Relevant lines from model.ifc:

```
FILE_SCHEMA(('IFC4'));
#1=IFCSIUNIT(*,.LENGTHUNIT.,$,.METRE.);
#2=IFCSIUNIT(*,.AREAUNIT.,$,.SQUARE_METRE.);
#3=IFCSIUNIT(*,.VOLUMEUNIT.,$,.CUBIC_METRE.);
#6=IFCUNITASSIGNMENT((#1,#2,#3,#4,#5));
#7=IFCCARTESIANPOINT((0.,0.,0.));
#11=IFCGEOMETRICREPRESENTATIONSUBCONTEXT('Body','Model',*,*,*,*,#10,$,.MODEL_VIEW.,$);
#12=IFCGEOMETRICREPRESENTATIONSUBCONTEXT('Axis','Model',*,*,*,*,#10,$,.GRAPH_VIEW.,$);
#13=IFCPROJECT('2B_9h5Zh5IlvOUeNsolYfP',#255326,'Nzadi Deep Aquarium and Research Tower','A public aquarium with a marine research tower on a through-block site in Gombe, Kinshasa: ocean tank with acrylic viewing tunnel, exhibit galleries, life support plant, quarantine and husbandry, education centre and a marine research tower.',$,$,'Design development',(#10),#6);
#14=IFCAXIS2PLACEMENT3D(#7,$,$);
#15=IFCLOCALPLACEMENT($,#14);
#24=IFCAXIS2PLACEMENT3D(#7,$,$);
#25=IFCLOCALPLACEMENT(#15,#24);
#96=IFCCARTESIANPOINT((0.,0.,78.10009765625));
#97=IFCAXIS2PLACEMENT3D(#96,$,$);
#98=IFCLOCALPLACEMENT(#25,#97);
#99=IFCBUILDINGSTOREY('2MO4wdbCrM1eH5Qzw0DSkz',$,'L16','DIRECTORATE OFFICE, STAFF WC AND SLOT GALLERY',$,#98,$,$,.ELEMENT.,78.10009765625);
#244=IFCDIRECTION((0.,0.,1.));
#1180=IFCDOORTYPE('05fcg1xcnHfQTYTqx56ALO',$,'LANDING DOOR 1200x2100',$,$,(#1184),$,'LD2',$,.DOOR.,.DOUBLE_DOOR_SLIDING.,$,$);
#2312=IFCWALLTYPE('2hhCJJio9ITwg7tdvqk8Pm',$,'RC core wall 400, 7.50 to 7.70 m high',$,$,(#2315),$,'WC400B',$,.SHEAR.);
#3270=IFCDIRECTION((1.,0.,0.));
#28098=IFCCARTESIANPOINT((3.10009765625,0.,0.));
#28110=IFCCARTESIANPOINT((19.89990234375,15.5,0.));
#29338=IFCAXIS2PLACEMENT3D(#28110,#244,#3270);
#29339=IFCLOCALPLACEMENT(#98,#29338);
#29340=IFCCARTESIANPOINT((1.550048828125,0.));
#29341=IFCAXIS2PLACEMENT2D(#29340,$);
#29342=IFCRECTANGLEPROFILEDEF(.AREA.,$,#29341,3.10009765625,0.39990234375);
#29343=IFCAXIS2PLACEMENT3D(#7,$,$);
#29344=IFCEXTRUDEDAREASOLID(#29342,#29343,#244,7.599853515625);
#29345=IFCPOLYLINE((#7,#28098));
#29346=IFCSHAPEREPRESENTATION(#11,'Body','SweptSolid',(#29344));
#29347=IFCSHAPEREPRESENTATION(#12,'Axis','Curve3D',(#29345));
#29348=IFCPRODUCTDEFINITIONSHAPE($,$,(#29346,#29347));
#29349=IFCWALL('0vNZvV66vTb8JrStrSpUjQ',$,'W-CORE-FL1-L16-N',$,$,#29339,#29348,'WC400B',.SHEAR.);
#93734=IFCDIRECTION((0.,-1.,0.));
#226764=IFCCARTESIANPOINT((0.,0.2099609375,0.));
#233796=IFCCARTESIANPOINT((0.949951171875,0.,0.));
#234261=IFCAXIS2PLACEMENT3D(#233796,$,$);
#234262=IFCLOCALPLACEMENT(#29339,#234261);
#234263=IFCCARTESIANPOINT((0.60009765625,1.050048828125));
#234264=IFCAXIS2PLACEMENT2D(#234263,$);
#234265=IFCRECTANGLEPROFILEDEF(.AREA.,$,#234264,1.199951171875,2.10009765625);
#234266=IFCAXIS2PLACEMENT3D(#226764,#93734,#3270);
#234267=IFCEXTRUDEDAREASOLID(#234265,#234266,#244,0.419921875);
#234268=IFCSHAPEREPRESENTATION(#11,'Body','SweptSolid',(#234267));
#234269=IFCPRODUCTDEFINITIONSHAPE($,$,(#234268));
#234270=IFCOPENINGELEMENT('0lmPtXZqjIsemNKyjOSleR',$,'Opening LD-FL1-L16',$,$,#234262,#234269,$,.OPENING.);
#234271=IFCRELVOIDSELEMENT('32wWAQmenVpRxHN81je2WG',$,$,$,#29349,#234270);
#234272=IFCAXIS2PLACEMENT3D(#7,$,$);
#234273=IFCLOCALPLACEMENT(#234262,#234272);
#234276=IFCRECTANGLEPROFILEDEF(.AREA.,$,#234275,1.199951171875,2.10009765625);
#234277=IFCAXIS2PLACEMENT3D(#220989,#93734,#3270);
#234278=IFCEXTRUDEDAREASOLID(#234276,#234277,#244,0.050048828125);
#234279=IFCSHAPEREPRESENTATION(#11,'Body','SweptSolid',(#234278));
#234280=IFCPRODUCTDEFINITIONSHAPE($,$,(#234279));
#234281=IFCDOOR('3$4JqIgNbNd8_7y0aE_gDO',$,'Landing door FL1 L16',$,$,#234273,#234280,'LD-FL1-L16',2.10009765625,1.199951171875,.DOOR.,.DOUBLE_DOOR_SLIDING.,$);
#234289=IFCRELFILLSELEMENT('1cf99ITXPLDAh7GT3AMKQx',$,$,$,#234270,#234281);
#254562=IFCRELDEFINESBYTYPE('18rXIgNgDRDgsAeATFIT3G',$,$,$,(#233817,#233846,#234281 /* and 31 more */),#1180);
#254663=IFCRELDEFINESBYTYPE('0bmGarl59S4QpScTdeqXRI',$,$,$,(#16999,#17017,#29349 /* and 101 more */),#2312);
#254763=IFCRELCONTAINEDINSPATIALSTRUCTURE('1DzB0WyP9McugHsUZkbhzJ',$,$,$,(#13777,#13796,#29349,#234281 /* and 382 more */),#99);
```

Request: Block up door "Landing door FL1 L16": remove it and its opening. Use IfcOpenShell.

```python
import ifcopenshell
import ifcopenshell.api.feature
import ifcopenshell.api.root
import ifcopenshell.geom
import ifcopenshell.util.shape

model = ifcopenshell.open("model.ifc")
settings = ifcopenshell.geom.settings()


def volume(element):
    """Net volume in cubic metres, openings subtracted."""
    shape = ifcopenshell.geom.create_shape(settings, element)
    return ifcopenshell.util.shape.get_volume(shape.geometry)


door = model.by_guid("3$4JqIgNbNd8_7y0aE_gDO")
opening = door.FillsVoids[0].RelatingOpeningElement
wall = opening.VoidsElements[0].RelatingBuildingElement
before = volume(wall)

ifcopenshell.api.root.remove_product(model, product=door)
ifcopenshell.api.feature.remove_feature(model, feature=opening)

after = volume(wall)

print(f"wall volume {before:.3f} -> {after:.3f} m3")

model.write("model-out.ifc")
```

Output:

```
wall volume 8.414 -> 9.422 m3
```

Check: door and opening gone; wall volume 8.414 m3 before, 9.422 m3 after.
